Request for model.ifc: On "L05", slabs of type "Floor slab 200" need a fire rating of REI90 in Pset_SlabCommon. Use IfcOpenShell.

First a look at what the model holds.

```python
import ifcopenshell
import ifcopenshell.util.element

model = ifcopenshell.open("model.ifc")
print(model.schema)
storey = next(s for s in model.by_type("IfcBuildingStorey") if s.Name == "L05")
slabs = [e for e in ifcopenshell.util.element.get_decomposition(storey) if e.is_a("IfcSlab")]
seen = {}
for e in slabs:
    element_type = ifcopenshell.util.element.get_type(e)
    key = (element_type.Name if element_type != e and element_type else None, ifcopenshell.util.element.get_pset(e, "Pset_SlabCommon", "FireRating"))
    seen[key] = seen.get(key, 0) + 1
for (name, value), count in sorted(seen.items(), key=str):
    print(count, "x", name, "|", value)
```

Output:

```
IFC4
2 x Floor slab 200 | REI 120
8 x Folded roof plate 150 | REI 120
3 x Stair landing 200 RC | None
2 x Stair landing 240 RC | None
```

```python
import ifcopenshell
import ifcopenshell.api.pset
import ifcopenshell.util.element

model = ifcopenshell.open("model.ifc")

storey = next(s for s in model.by_type("IfcBuildingStorey") if s.Name == "L05")
slabs = [e for e in ifcopenshell.util.element.get_decomposition(storey) if e.is_a("IfcSlab")]

count = 0
for e in slabs:
    element_type = ifcopenshell.util.element.get_type(e)
    if element_type in (None, e) or element_type.Name != "Floor slab 200":
        continue
    # add_pset returns the element's existing set when there is one.
    pset = ifcopenshell.api.pset.add_pset(model, product=e, name="Pset_SlabCommon")
    ifcopenshell.api.pset.edit_pset(model, pset=pset, properties={"FireRating": "REI90"})
    count += 1

print(count, "slabs updated")

model.write("model_rev.ifc")
```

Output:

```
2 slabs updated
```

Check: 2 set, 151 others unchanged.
